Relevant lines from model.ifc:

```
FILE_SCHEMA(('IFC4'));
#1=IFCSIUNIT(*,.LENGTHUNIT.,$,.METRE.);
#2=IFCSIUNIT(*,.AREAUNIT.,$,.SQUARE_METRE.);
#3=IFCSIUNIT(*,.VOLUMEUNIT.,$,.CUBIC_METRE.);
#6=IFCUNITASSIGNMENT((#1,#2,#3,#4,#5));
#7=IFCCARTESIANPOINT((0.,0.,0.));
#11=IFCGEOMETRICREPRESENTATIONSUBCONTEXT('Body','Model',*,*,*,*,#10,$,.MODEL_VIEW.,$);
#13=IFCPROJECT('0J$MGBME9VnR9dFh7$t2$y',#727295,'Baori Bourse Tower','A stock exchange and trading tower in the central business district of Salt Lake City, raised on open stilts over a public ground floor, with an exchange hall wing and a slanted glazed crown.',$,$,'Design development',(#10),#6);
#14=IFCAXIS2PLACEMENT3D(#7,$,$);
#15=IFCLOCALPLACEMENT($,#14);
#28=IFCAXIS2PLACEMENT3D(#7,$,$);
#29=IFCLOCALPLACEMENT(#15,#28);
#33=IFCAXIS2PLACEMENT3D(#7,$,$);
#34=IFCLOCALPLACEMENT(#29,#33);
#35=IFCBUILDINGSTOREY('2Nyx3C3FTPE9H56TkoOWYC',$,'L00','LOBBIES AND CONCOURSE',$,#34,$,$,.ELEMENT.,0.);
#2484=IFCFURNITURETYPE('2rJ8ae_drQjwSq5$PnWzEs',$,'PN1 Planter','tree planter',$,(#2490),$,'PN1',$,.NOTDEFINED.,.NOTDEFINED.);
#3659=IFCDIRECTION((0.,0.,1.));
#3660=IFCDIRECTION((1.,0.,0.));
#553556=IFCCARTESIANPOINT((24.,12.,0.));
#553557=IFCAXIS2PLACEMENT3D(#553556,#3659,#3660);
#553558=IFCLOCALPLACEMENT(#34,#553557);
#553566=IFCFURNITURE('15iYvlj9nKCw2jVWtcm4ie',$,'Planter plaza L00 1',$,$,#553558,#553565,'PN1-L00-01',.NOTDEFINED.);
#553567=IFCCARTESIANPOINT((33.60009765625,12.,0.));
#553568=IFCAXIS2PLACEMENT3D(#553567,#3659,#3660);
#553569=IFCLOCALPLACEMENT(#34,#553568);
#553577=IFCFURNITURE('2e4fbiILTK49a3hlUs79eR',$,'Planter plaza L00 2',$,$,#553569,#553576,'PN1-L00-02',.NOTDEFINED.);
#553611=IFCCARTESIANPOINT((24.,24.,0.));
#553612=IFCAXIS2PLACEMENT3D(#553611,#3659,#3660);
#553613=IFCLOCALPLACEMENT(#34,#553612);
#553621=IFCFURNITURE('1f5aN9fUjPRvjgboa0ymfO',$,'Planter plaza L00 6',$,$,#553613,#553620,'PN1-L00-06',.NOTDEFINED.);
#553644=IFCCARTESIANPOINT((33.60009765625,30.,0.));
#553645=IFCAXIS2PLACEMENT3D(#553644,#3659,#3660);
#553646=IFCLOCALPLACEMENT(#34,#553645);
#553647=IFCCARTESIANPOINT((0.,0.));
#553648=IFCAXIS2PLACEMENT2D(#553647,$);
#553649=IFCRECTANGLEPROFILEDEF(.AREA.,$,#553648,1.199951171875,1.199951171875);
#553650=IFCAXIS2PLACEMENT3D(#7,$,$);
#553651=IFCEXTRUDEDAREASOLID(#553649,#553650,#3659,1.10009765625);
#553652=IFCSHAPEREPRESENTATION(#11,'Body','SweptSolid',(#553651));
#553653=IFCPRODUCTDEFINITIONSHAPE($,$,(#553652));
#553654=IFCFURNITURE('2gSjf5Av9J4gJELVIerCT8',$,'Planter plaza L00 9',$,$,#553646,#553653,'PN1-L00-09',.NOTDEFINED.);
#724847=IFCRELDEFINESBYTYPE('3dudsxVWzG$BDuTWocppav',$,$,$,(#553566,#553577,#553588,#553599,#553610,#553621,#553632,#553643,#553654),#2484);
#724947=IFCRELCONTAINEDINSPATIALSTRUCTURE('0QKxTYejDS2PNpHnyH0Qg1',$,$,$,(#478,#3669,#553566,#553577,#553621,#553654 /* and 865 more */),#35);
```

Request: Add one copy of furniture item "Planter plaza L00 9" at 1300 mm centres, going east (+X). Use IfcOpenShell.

```python
import numpy as np
import ifcopenshell
import ifcopenshell.api.geometry
import ifcopenshell.api.root
import ifcopenshell.util.element
import ifcopenshell.util.placement

model = ifcopenshell.open("model.ifc")

source = model.by_id(553654)
base = ifcopenshell.util.placement.get_local_placement(source.ObjectPlacement)
step = np.array([1.0, 0.0, 0.0]) * 1.3

for i in range(1, 2):
    copy = ifcopenshell.api.root.copy_class(model, product=source)
    copy.Representation = ifcopenshell.util.element.copy_deep(
        model, source.Representation, exclude=["IfcGeometricRepresentationContext", "IfcRepresentationMap"]
    )
    copy.Tag = None
    matrix = base.copy()
    matrix[:3, 3] += i * step
    print("added at", matrix[:3, 3].round(3) + 0.0)
    ifcopenshell.api.geometry.edit_object_placement(model, product=copy, matrix=matrix, is_si=False)

model.write("model_rev.ifc")
```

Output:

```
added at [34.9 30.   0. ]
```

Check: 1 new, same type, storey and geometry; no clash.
